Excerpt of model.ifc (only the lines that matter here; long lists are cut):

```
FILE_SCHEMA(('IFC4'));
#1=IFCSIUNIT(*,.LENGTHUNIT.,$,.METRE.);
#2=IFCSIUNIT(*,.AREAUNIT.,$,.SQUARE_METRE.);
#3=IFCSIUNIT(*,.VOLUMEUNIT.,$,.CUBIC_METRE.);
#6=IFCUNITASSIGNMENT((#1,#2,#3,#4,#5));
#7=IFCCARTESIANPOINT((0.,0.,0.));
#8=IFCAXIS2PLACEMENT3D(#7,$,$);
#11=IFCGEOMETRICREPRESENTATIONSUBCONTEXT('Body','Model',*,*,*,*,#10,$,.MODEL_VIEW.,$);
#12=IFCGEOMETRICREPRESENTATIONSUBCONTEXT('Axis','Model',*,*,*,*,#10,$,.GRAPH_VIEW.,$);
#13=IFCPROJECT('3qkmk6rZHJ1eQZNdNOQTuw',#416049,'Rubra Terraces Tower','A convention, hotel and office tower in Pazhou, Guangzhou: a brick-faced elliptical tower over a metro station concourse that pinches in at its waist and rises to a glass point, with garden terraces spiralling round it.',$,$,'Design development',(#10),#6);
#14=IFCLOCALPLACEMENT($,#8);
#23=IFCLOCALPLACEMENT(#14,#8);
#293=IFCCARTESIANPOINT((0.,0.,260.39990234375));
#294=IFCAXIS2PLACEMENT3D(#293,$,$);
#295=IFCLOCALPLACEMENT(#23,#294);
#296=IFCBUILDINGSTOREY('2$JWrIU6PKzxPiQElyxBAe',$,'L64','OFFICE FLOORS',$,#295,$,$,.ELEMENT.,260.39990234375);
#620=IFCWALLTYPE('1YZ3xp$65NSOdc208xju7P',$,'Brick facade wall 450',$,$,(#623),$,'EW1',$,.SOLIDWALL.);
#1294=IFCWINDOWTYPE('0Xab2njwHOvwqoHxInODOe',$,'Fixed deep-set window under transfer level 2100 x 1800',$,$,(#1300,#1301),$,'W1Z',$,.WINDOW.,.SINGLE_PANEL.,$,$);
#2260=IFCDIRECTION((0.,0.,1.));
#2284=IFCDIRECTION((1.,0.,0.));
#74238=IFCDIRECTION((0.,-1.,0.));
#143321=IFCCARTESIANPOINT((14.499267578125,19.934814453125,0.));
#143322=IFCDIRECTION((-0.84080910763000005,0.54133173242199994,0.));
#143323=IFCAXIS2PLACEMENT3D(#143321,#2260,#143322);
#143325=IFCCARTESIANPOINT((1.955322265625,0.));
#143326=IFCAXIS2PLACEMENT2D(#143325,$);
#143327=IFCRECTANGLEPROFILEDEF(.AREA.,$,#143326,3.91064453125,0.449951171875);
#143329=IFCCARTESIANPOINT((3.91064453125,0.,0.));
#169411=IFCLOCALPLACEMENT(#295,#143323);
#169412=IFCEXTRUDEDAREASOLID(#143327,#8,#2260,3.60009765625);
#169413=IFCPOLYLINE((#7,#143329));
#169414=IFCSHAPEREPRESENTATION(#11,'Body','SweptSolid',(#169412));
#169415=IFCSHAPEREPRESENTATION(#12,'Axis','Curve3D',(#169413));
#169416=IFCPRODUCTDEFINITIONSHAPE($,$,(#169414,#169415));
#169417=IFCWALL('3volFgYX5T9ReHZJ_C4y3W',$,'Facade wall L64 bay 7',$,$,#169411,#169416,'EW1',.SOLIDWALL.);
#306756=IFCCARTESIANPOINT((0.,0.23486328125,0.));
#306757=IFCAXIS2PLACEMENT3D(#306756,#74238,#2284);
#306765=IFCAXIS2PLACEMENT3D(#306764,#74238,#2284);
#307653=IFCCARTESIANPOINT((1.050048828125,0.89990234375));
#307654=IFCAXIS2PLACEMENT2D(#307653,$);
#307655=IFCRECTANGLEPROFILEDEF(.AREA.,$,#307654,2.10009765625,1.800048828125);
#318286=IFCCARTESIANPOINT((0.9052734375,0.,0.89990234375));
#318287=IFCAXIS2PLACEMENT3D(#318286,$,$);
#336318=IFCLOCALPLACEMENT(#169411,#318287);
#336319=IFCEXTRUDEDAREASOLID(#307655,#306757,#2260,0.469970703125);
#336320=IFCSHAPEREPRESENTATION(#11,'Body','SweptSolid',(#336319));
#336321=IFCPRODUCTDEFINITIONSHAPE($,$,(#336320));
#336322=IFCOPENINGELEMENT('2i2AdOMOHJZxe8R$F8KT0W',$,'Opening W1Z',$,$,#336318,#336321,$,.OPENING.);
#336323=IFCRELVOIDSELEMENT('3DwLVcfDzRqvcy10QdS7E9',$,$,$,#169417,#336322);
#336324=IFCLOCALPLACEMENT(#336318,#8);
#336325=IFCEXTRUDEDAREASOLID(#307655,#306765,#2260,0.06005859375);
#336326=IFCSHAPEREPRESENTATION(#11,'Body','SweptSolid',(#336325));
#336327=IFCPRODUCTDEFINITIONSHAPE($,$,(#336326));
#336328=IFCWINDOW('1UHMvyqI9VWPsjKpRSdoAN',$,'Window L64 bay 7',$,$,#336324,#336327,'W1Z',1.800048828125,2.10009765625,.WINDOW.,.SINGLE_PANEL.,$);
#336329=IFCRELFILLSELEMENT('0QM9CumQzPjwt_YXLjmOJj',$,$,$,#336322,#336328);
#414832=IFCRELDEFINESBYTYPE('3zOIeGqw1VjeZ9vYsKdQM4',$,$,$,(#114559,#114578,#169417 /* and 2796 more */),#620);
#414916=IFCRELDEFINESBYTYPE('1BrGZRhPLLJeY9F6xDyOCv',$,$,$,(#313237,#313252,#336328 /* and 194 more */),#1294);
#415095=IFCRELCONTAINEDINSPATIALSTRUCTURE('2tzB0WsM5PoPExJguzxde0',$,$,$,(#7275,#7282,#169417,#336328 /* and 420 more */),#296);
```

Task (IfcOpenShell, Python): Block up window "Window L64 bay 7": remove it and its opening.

```python
import ifcopenshell
import ifcopenshell.api.feature
import ifcopenshell.api.root
import ifcopenshell.geom
import ifcopenshell.util.shape

model = ifcopenshell.open("model.ifc")
settings = ifcopenshell.geom.settings()


def volume(element):
    """Net volume in cubic metres, openings subtracted."""
    shape = ifcopenshell.geom.create_shape(settings, element)
    return ifcopenshell.util.shape.get_volume(shape.geometry)


window = model.by_guid("1UHMvyqI9VWPsjKpRSdoAN")
opening = window.FillsVoids[0].RelatingOpeningElement
wall = opening.VoidsElements[0].RelatingBuildingElement
before = volume(wall)

ifcopenshell.api.root.remove_product(model, product=window)
ifcopenshell.api.feature.remove_feature(model, feature=opening)

after = volume(wall)

print(f"wall volume {before:.3f} -> {after:.3f} m3")

model.write("model_rev.ifc")
```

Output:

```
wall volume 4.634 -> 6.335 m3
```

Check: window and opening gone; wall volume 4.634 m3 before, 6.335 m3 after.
